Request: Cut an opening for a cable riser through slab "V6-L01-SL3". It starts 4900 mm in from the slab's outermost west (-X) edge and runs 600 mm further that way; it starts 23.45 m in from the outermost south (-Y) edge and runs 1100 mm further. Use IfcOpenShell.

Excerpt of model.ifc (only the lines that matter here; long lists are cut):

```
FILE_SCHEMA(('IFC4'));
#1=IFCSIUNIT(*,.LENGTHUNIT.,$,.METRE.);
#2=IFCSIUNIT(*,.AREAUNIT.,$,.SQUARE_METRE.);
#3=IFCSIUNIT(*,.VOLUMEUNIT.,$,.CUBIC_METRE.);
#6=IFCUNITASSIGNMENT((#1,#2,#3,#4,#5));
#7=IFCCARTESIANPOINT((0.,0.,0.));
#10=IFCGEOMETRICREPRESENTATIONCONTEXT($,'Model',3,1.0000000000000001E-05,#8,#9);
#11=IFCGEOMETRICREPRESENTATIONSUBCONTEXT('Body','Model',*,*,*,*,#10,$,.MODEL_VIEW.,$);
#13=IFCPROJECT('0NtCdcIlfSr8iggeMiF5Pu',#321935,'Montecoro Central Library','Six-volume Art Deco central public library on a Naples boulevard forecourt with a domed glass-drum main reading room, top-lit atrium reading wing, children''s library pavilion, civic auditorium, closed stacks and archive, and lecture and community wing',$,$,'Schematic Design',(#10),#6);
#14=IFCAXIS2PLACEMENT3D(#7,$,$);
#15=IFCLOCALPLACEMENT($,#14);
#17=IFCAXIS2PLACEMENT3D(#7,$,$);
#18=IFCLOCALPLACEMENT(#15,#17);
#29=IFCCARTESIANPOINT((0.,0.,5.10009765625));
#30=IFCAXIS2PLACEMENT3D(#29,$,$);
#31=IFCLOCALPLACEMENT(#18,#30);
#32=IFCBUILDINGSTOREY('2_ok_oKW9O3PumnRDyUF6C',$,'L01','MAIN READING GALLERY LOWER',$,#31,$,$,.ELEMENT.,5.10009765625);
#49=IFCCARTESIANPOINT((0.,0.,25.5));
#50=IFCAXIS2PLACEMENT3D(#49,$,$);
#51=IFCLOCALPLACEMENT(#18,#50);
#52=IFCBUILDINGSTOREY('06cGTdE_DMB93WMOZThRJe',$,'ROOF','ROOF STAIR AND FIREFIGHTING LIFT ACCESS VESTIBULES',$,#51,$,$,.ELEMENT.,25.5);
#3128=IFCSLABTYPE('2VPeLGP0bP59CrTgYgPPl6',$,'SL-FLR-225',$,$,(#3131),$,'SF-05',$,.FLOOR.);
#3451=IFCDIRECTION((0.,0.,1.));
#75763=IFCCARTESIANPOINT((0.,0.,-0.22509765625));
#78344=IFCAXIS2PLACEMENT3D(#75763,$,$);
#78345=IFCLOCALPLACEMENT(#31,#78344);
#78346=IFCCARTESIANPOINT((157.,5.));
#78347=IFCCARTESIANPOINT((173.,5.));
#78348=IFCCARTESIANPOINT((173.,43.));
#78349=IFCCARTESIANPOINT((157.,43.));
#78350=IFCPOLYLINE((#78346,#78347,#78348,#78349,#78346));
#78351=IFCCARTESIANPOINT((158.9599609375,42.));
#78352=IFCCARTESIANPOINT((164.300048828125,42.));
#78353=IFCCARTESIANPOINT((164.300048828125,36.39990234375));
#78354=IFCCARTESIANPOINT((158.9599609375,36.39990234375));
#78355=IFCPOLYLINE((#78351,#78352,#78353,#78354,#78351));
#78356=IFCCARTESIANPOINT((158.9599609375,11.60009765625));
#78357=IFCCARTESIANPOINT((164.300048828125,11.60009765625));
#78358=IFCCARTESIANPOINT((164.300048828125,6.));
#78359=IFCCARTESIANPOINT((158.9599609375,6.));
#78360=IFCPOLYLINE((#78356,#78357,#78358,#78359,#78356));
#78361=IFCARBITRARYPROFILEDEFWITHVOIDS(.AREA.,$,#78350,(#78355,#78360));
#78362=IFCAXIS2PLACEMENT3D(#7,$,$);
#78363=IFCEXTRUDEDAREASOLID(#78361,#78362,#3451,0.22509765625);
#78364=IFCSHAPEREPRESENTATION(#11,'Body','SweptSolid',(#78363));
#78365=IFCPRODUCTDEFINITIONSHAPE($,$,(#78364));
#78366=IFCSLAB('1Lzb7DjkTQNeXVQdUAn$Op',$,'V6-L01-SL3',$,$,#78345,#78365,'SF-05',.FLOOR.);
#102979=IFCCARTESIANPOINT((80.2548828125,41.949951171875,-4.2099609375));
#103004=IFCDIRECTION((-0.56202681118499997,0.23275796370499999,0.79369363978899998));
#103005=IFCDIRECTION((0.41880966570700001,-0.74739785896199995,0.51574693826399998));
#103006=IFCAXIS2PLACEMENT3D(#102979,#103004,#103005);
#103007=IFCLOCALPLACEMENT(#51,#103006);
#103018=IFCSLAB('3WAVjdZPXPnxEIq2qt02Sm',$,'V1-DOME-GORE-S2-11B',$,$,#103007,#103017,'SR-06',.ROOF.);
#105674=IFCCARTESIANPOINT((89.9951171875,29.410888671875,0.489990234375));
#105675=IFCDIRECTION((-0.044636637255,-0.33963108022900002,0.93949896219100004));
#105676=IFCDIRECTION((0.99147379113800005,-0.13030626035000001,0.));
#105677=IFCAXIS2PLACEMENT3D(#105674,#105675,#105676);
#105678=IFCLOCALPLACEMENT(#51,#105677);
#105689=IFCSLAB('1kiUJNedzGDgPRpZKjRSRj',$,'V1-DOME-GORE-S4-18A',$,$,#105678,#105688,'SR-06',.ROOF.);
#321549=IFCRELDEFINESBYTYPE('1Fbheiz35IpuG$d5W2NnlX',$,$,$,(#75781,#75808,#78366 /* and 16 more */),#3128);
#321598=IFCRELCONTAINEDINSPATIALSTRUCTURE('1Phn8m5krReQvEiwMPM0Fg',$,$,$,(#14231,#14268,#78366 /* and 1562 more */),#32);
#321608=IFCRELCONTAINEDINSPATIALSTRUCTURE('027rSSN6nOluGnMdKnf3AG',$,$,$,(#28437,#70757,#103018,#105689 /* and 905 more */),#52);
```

```python
import numpy as np
import ifcopenshell
import ifcopenshell.api.feature
import ifcopenshell.api.geometry
import ifcopenshell.api.root
import ifcopenshell.geom
import ifcopenshell.util.placement
import ifcopenshell.util.representation
import ifcopenshell.util.shape
import ifcopenshell.util.unit

model = ifcopenshell.open("model.ifc")
unit_scale = ifcopenshell.util.unit.calculate_unit_scale(model)
settings = ifcopenshell.geom.settings()


def volume(element):
    """Net volume in cubic metres, openings subtracted."""
    shape = ifcopenshell.geom.create_shape(settings, element)
    return ifcopenshell.util.shape.get_volume(shape.geometry)


slab = model.by_guid("1Lzb7DjkTQNeXVQdUAn$Op")
before = volume(slab)

# Extent in the slab's own axes, in metres. The edges named are its -X and -Y sides.
slab_shape = ifcopenshell.geom.create_shape(settings, slab)
vertices = ifcopenshell.util.shape.get_vertices(slab_shape.geometry)
x_min, y_min, bottom = vertices.min(axis=0)
top = vertices[:, 2].max()

opening = ifcopenshell.api.root.create_entity(model, ifc_class="IfcOpeningElement", name="Cable riser opening", predefined_type="OPENING")
context = ifcopenshell.util.representation.get_context(model, "Model", "Body", "MODEL_VIEW")
width, depth = 0.6, 1.1
outline = [(0.0, 0.0), (width, 0.0), (width, depth), (0.0, depth), (0.0, 0.0)]
# Overshoot both faces by 50 mm so the cut is clean.
shape = ifcopenshell.api.geometry.add_slab_representation(
    model, context=context, depth=top - bottom + 0.1, polyline=outline
)
ifcopenshell.api.geometry.assign_representation(model, product=opening, representation=shape)

matrix = ifcopenshell.util.placement.get_local_placement(slab.ObjectPlacement)
matrix[:, 3] = matrix @ np.append(np.array([x_min + 4.9, y_min + 23.45, bottom - 0.05]) / unit_scale, 1.0)
ifcopenshell.api.geometry.edit_object_placement(model, product=opening, matrix=matrix, is_si=False)
ifcopenshell.api.feature.add_feature(model, feature=opening, element=slab)

after = volume(slab)

print(f"slab volume {before:.3f} -> {after:.3f} m3")

model.write("model_rev.ifc")
```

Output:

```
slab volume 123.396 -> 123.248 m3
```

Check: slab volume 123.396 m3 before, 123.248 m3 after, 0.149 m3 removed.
